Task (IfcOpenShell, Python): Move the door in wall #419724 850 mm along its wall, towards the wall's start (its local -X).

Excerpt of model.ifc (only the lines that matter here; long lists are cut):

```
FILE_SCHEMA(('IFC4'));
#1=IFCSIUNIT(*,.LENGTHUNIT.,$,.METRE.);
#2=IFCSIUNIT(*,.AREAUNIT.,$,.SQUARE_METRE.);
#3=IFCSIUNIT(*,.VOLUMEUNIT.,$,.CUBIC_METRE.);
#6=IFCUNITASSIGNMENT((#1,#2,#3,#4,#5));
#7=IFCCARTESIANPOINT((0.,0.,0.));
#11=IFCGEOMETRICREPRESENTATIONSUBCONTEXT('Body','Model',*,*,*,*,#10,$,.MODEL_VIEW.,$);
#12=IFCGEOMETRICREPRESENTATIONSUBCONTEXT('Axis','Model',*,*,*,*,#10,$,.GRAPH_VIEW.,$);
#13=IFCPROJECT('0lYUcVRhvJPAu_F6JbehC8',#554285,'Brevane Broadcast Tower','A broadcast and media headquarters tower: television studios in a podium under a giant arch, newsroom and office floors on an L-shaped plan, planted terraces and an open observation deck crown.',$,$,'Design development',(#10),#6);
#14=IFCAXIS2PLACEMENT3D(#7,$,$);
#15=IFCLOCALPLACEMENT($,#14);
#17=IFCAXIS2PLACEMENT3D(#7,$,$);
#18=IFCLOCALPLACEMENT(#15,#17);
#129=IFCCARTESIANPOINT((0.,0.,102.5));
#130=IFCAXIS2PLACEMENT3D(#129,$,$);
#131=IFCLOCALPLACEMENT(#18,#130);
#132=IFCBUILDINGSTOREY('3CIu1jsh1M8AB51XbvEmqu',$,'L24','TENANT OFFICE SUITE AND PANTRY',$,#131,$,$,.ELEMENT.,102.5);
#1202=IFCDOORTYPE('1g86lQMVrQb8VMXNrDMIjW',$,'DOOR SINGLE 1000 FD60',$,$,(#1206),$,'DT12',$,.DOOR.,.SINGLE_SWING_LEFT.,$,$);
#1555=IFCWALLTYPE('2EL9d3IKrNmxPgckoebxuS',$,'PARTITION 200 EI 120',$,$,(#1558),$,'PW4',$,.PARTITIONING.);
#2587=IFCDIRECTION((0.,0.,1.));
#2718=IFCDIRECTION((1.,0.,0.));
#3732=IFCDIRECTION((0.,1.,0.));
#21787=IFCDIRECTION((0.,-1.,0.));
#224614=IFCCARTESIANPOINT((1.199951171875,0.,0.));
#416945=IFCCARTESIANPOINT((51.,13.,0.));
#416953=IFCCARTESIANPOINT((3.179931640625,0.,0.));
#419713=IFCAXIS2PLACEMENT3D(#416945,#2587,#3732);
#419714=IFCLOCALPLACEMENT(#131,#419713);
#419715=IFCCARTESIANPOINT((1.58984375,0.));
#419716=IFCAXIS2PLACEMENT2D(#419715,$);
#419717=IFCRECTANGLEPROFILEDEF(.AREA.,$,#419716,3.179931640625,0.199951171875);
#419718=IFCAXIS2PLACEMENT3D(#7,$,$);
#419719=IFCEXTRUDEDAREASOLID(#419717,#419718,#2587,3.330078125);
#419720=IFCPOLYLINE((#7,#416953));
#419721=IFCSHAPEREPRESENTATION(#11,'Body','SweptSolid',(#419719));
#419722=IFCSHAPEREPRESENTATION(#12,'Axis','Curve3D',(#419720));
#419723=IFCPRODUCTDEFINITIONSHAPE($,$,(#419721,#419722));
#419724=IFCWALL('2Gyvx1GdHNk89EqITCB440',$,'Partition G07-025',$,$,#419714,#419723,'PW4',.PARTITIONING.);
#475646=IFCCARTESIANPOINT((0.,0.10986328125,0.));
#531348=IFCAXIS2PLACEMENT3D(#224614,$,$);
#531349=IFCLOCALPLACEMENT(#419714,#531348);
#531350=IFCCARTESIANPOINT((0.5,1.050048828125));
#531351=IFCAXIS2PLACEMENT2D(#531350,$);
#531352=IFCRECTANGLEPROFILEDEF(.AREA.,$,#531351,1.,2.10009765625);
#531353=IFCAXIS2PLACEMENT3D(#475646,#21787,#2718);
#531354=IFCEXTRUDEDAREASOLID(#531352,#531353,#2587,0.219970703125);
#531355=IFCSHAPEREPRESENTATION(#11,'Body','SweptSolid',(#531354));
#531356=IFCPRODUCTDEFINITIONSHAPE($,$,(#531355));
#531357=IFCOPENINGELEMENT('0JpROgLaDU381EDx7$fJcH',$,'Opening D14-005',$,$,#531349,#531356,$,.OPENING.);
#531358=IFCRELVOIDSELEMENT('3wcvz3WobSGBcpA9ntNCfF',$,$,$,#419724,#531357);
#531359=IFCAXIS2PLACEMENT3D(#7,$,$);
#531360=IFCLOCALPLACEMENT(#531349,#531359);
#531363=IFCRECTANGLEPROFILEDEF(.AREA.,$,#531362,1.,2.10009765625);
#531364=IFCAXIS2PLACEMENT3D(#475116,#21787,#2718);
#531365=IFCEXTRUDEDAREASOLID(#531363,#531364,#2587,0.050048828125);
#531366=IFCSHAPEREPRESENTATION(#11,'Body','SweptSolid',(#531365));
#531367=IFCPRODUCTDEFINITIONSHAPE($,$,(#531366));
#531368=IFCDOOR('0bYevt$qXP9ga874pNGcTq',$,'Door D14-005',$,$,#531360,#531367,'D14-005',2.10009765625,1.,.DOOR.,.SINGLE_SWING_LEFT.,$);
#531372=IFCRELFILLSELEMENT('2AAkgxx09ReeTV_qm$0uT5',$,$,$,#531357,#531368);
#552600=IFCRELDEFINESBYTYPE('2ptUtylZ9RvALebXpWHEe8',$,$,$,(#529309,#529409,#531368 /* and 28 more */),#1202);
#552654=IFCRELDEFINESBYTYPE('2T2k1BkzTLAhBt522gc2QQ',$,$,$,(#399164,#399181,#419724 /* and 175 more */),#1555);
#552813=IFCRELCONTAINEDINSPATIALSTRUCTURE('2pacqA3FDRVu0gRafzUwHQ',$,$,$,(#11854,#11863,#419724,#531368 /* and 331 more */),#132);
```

```python
import ifcopenshell
import ifcopenshell.api.geometry
import ifcopenshell.util.placement
import ifcopenshell.util.unit

model = ifcopenshell.open("model.ifc")
unit_scale = ifcopenshell.util.unit.calculate_unit_scale(model)

door = model.by_guid("0bYevt$qXP9ga874pNGcTq")
opening = door.FillsVoids[0].RelatingOpeningElement
wall = opening.VoidsElements[0].RelatingBuildingElement

wall_matrix = ifcopenshell.util.placement.get_local_placement(wall.ObjectPlacement)
shift = wall_matrix[:3, 0] * -0.85 / unit_scale
before = ifcopenshell.util.placement.get_local_placement(door.ObjectPlacement)[:3, 3].copy()

# The door is placed relative to its opening, so it follows when the opening moves.
matrix = ifcopenshell.util.placement.get_local_placement(opening.ObjectPlacement)
matrix[:3, 3] += shift
ifcopenshell.api.geometry.edit_object_placement(
    model, product=opening, matrix=matrix, is_si=False, should_transform_children=True
)

after = ifcopenshell.util.placement.get_local_placement(door.ObjectPlacement)[:3, 3]
print("door moved by", (after - before).round(3) + 0.0)

model.write("model-out.ifc")
```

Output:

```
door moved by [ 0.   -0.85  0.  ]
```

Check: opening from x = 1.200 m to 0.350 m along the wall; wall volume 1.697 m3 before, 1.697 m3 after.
